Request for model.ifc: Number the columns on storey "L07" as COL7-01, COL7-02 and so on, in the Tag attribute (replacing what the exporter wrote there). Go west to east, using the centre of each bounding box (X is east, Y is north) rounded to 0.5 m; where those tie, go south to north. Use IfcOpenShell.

First a look at what the model holds.

```python
import ifcopenshell
import ifcopenshell.util.element
import ifcopenshell.util.placement

model = ifcopenshell.open("model.ifc")
print(model.schema)
storey = next(s for s in model.by_type("IfcBuildingStorey") if s.Name == "L07")
columns = [e for e in ifcopenshell.util.element.get_decomposition(storey) if e.is_a("IfcColumn")]
for e in sorted(columns, key=lambda e: e.id()):
    origin = ifcopenshell.util.placement.get_local_placement(e.ObjectPlacement)[:3, 3]
    print(e.id(), e.Tag, e.Name, origin.round(2) + 0.0, sep=" | ")
```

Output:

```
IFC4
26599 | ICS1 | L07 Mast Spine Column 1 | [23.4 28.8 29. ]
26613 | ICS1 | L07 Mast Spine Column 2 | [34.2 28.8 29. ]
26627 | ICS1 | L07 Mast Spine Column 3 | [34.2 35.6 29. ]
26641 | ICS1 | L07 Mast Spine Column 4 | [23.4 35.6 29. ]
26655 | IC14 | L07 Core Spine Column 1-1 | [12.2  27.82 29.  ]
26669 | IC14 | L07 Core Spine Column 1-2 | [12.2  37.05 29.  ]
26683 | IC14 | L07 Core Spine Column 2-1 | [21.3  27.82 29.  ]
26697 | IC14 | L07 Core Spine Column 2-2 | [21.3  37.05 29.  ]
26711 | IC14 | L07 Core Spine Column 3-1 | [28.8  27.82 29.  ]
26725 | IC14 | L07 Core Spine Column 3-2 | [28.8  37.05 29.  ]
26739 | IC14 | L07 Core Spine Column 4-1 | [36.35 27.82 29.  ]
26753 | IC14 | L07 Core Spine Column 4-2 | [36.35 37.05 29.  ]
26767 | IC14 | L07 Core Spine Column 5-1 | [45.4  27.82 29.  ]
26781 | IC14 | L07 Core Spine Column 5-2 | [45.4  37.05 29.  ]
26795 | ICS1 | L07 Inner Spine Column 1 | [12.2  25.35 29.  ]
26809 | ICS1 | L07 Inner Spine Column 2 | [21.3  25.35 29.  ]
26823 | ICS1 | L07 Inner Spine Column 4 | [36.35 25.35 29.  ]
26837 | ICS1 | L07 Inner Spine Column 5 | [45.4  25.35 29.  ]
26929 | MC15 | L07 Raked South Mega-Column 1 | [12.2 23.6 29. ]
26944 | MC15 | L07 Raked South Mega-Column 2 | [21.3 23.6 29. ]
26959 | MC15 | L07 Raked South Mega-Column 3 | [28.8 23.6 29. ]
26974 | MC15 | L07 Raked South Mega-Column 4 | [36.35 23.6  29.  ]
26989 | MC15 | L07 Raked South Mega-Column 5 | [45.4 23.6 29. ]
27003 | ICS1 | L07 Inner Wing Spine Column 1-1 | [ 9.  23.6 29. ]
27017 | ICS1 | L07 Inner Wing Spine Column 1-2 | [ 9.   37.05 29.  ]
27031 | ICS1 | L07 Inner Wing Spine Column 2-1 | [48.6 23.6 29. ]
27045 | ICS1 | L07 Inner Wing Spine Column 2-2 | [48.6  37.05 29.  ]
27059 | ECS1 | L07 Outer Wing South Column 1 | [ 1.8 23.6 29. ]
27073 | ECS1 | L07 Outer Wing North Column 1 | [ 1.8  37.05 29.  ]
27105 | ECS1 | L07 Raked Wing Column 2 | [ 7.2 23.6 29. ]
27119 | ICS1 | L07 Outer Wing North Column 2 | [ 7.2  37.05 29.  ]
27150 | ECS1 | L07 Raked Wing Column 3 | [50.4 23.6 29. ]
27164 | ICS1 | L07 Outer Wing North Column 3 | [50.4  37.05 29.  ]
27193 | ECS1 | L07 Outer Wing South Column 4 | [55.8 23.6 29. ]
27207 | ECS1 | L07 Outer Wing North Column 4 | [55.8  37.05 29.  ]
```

```python
import ifcopenshell
import ifcopenshell.geom
import ifcopenshell.util.element
import ifcopenshell.util.shape

model = ifcopenshell.open("model.ifc")
settings = ifcopenshell.geom.settings()
settings.set("use-world-coords", True)


def centre(element):
    shape = ifcopenshell.geom.create_shape(settings, element)
    return ifcopenshell.util.shape.get_bbox_centroid(shape.geometry)


storey = next(s for s in model.by_type("IfcBuildingStorey") if s.Name == "L07")
columns = [e for e in ifcopenshell.util.element.get_decomposition(storey) if e.is_a("IfcColumn")]

# Insertion points can sit at a corner or the storey origin, so sort by the geometry (in metres).
centres = {e: centre(e) for e in columns}
columns.sort(key=lambda e: (round(centres[e][0] / 0.5), centres[e][1]))

for i, e in enumerate(columns, start=1):
    number = f"COL7-{i:02d}"
    e.Tag = number
    print(e.id(), number)

model.write("model_v2.ifc")
```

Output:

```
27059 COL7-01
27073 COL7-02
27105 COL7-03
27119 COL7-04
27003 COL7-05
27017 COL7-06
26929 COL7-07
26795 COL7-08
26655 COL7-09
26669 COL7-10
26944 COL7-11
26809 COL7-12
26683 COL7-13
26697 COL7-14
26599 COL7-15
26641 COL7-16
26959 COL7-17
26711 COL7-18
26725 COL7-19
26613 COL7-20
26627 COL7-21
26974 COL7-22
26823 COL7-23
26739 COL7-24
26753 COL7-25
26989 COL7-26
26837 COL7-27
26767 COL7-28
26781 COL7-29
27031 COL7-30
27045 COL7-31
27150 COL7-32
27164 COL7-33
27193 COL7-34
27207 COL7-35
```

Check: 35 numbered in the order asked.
